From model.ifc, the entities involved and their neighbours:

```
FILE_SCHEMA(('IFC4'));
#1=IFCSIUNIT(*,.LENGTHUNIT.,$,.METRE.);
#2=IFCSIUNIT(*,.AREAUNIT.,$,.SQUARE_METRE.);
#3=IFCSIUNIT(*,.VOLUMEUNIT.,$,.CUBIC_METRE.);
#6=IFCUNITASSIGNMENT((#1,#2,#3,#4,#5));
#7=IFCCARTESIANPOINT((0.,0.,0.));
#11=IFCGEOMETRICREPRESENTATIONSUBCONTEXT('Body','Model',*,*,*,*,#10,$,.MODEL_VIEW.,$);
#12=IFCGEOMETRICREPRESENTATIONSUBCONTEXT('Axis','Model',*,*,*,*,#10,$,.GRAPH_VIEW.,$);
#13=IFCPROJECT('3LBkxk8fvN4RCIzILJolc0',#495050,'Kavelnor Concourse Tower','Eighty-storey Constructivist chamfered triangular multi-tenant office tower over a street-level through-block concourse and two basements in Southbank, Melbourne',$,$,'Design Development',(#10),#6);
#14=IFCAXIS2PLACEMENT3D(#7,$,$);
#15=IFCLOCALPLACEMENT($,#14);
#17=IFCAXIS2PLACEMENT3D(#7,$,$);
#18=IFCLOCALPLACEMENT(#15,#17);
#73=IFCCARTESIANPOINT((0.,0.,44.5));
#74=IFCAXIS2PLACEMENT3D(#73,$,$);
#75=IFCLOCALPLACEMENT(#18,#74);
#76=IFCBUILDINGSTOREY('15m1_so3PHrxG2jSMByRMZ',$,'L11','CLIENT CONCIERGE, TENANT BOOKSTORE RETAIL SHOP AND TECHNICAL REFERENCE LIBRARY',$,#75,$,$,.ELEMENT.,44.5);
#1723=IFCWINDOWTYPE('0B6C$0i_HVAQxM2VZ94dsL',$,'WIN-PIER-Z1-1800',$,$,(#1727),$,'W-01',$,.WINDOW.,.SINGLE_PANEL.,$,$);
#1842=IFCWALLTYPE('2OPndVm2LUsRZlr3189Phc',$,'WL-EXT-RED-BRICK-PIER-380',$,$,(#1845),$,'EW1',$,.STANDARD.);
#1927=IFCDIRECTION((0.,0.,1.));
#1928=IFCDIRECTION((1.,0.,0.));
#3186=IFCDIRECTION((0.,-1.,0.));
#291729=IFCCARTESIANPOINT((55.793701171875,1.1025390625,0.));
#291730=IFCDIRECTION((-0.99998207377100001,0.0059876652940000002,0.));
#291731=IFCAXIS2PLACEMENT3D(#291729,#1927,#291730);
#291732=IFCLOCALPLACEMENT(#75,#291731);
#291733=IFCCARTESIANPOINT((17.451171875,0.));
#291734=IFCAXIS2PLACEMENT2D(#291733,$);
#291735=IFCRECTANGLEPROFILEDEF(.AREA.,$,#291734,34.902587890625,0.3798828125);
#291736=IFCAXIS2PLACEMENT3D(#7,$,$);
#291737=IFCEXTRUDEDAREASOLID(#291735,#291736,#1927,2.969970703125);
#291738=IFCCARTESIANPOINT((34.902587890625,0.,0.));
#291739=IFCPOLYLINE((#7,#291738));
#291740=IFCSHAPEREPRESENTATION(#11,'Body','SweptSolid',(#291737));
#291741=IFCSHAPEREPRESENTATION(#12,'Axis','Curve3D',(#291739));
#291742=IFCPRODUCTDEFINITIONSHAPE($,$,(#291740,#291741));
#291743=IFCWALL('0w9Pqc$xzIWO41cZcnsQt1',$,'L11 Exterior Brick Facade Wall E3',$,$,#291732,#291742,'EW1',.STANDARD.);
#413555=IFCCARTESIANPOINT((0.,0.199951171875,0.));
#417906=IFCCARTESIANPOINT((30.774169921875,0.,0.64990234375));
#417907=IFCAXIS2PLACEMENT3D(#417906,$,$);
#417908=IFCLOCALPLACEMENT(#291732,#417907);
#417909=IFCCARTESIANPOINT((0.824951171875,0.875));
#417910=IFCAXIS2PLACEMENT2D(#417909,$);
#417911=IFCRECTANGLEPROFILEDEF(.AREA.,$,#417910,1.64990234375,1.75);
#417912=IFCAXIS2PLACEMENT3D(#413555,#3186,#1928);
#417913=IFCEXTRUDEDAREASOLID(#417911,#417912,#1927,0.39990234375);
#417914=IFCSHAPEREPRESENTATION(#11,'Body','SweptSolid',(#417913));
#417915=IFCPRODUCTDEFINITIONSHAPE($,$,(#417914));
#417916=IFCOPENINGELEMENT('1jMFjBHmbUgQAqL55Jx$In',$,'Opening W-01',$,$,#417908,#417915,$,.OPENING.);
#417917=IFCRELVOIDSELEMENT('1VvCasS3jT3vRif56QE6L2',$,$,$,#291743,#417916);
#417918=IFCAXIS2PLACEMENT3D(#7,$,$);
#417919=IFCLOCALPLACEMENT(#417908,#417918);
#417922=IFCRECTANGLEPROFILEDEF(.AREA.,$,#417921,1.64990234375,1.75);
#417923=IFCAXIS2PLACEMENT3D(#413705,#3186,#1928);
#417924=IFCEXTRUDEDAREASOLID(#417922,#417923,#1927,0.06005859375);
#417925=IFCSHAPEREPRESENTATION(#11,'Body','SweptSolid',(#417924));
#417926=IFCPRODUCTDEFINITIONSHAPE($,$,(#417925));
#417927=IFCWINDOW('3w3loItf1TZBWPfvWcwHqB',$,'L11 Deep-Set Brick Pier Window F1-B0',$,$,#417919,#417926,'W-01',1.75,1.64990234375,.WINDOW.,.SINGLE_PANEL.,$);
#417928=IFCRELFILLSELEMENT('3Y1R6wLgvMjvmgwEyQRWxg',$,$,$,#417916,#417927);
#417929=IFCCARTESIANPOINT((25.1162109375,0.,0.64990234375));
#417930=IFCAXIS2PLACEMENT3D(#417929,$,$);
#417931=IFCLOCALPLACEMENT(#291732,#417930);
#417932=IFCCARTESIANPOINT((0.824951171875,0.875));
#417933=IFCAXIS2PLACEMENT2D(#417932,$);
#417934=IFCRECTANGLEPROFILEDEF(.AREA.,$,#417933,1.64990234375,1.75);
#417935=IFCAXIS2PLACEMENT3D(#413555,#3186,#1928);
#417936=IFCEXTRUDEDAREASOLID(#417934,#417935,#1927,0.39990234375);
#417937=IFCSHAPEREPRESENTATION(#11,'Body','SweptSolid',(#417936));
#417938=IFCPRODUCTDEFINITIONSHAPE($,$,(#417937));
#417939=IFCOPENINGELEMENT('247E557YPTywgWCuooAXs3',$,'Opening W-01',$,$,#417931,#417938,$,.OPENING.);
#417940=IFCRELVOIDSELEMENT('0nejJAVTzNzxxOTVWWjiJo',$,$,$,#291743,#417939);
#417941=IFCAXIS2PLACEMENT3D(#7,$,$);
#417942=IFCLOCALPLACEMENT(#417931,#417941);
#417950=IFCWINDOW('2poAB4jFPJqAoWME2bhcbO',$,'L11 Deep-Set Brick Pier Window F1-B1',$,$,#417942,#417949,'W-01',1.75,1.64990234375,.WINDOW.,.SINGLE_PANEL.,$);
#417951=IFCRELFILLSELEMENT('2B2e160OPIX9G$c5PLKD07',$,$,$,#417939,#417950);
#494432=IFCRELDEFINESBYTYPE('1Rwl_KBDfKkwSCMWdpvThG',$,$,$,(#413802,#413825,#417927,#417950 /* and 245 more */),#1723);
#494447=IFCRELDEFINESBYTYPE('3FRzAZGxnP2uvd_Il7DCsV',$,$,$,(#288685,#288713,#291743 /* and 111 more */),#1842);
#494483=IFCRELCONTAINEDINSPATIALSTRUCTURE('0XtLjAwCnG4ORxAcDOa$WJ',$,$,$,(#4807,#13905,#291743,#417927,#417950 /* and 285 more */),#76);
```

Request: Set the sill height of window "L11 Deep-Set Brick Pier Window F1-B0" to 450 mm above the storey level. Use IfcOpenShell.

```python
import numpy as np
import ifcopenshell
import ifcopenshell.api.geometry
import ifcopenshell.geom
import ifcopenshell.util.element
import ifcopenshell.util.placement
import ifcopenshell.util.shape
import ifcopenshell.util.unit

model = ifcopenshell.open("model.ifc")
unit_scale = ifcopenshell.util.unit.calculate_unit_scale(model)

window = model.by_guid("3w3loItf1TZBWPfvWcwHqB")
opening = window.FillsVoids[0].RelatingOpeningElement
storey = ifcopenshell.util.element.get_container(window, ifc_class="IfcBuildingStorey")
level = ifcopenshell.util.placement.get_local_placement(storey.ObjectPlacement)[2, 3]

# The opening's origin need not be at the sill, so measure its lowest point.
shape = ifcopenshell.geom.create_shape(ifcopenshell.geom.settings(), opening)
bottom = ifcopenshell.util.shape.get_shape_bottom_elevation(shape, shape.geometry) / unit_scale
dz = level + 0.45 / unit_scale - bottom

shift = np.array([0.0, 0.0, dz])
# The window is placed relative to its opening, so it follows when the opening moves.
matrix = ifcopenshell.util.placement.get_local_placement(opening.ObjectPlacement)
matrix[:3, 3] += shift
ifcopenshell.api.geometry.edit_object_placement(
    model, product=opening, matrix=matrix, is_si=False, should_transform_children=True
)

print(f"moved by {dz * unit_scale:+.3f} m")

model.write("model_v2.ifc")
```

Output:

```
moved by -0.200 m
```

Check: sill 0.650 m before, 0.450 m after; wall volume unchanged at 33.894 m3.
